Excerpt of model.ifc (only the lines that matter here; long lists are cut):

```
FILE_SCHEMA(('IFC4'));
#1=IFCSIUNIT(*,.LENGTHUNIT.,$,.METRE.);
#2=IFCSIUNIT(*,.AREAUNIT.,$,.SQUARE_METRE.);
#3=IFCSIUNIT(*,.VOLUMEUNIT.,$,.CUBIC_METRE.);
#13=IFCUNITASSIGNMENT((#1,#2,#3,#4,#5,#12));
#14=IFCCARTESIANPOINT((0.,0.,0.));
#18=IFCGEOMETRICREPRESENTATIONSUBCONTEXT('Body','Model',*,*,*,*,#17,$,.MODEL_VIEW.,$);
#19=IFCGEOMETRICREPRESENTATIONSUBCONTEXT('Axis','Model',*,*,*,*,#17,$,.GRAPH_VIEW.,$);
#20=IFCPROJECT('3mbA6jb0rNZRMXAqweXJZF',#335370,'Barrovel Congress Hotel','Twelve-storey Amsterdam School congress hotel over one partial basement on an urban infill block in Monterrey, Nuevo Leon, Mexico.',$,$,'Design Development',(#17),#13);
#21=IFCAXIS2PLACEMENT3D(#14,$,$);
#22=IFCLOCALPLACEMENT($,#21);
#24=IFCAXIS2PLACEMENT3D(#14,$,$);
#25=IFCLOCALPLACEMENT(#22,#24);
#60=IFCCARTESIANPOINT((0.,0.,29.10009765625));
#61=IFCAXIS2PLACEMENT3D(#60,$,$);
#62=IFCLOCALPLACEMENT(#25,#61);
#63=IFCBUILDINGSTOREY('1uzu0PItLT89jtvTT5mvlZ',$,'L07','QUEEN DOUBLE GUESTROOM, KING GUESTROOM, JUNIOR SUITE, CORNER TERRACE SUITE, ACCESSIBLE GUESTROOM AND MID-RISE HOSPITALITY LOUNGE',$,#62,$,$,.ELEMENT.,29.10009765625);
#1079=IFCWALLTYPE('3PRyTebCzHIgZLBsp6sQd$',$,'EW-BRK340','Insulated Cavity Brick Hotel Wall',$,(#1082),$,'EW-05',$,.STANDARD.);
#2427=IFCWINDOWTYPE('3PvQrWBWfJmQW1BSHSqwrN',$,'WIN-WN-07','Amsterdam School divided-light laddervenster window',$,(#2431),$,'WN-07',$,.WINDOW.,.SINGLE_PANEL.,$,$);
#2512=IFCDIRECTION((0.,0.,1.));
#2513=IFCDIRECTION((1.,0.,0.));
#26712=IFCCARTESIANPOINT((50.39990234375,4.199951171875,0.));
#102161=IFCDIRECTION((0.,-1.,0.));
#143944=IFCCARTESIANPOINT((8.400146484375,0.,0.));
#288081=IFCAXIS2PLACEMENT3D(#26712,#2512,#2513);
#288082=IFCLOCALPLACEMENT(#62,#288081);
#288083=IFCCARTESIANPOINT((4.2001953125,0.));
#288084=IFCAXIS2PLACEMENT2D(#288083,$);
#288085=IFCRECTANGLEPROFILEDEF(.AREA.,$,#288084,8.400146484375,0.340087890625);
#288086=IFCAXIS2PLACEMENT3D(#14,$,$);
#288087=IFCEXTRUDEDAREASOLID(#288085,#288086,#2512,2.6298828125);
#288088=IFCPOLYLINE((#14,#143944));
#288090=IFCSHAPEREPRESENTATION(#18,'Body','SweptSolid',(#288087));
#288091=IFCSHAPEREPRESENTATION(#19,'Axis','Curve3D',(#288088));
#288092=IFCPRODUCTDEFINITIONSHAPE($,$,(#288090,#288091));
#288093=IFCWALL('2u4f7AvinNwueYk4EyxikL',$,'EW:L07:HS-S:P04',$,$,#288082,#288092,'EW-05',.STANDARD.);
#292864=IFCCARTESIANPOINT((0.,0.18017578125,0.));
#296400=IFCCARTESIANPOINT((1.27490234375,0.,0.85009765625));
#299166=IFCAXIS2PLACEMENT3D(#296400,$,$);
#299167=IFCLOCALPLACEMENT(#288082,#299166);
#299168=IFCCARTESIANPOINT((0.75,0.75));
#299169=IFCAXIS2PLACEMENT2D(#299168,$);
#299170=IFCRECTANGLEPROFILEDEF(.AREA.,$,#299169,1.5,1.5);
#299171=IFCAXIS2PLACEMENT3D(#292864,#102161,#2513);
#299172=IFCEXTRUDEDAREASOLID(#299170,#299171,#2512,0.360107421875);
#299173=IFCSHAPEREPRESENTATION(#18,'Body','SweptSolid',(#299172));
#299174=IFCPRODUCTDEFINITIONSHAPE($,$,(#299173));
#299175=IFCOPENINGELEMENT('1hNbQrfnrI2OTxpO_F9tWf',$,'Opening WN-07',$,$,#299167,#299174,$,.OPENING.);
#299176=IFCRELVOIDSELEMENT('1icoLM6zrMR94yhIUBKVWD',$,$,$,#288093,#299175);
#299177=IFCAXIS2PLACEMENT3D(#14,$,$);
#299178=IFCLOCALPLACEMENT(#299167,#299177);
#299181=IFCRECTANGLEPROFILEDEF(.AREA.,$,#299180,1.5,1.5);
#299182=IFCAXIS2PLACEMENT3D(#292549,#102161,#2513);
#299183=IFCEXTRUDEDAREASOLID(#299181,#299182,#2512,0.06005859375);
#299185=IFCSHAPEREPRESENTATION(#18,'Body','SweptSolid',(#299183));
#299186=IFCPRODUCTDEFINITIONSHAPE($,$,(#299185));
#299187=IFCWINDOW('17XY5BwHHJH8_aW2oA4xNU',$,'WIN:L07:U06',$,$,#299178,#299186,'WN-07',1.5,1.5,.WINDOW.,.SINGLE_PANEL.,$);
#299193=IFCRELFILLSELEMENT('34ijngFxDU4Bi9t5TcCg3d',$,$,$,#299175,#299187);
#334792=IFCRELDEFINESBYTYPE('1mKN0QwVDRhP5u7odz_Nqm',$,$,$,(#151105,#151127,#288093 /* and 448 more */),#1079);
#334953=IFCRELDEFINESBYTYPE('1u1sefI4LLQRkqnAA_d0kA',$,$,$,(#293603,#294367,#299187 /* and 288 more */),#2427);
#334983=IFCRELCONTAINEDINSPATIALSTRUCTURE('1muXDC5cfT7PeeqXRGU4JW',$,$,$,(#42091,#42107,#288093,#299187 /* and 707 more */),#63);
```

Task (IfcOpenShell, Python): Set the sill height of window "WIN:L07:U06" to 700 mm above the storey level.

```python
import numpy as np
import ifcopenshell
import ifcopenshell.api.geometry
import ifcopenshell.geom
import ifcopenshell.util.element
import ifcopenshell.util.placement
import ifcopenshell.util.shape
import ifcopenshell.util.unit

model = ifcopenshell.open("model.ifc")
unit_scale = ifcopenshell.util.unit.calculate_unit_scale(model)

window = model.by_guid("17XY5BwHHJH8_aW2oA4xNU")
opening = window.FillsVoids[0].RelatingOpeningElement
storey = ifcopenshell.util.element.get_container(window, ifc_class="IfcBuildingStorey")
level = ifcopenshell.util.placement.get_local_placement(storey.ObjectPlacement)[2, 3]

# The opening's origin need not be at the sill, so measure its lowest point.
shape = ifcopenshell.geom.create_shape(ifcopenshell.geom.settings(), opening)
bottom = ifcopenshell.util.shape.get_shape_bottom_elevation(shape, shape.geometry) / unit_scale
dz = level + 0.7 / unit_scale - bottom

shift = np.array([0.0, 0.0, dz])
# The window is placed relative to its opening, so it follows when the opening moves.
matrix = ifcopenshell.util.placement.get_local_placement(opening.ObjectPlacement)
matrix[:3, 3] += shift
ifcopenshell.api.geometry.edit_object_placement(
    model, product=opening, matrix=matrix, is_si=False, should_transform_children=True
)

print(f"moved by {dz * unit_scale:+.3f} m")

model.write("model_rev.ifc")
```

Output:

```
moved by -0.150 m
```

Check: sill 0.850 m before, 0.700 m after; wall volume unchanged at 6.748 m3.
